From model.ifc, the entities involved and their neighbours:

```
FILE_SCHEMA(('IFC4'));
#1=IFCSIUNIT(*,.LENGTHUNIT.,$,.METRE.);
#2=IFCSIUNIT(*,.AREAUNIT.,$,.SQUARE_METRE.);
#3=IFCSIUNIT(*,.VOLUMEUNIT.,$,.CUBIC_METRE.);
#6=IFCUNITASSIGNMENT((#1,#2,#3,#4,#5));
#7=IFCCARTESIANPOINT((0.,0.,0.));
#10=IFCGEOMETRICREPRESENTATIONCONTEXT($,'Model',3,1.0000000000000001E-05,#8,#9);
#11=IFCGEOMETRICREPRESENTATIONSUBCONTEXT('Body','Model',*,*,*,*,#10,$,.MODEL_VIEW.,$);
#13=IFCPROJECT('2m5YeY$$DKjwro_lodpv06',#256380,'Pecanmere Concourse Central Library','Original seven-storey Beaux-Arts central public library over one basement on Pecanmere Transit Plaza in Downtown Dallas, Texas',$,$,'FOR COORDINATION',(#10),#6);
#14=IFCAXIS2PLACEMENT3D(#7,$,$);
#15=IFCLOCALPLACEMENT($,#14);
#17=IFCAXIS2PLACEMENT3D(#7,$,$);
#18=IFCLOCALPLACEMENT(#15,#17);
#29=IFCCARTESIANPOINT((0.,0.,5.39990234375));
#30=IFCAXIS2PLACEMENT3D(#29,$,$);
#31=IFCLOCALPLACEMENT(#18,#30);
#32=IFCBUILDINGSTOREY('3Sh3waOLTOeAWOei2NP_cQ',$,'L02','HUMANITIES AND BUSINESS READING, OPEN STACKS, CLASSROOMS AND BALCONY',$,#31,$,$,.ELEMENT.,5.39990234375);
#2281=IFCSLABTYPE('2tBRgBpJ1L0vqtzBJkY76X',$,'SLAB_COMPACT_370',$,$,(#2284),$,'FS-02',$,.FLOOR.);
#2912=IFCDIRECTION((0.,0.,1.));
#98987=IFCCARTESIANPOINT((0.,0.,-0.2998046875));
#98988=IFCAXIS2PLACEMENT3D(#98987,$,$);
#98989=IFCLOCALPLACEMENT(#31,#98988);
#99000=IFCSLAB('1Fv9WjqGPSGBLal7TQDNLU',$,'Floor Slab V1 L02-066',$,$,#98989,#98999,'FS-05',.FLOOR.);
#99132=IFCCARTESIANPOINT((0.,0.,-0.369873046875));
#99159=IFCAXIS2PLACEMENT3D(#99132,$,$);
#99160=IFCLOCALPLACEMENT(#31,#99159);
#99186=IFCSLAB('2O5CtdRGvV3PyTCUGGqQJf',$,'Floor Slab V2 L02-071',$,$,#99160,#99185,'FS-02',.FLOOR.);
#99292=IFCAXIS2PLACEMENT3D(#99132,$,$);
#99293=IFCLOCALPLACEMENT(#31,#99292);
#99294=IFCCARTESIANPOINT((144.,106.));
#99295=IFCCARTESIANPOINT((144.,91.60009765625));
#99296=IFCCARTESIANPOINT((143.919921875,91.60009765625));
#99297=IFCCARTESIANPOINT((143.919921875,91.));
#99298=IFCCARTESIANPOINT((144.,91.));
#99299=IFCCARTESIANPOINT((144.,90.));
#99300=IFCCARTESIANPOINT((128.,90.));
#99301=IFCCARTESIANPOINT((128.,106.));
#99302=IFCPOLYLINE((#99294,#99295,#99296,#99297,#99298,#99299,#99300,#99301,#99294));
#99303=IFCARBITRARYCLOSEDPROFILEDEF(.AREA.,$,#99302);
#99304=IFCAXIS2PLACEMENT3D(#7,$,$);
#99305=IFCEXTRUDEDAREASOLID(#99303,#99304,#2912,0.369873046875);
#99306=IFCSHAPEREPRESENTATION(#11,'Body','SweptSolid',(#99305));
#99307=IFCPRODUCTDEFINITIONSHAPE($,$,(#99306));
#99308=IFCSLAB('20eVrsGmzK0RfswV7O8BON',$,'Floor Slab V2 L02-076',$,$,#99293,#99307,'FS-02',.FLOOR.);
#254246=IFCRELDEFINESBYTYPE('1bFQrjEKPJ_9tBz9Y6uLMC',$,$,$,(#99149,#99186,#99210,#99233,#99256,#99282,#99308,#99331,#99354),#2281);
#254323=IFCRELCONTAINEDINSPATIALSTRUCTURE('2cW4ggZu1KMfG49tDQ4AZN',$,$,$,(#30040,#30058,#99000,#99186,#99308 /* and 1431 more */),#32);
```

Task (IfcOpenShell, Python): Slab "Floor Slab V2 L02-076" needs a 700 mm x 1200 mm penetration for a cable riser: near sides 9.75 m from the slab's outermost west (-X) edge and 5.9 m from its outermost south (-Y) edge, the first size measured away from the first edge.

```python
import numpy as np
import ifcopenshell
import ifcopenshell.api.feature
import ifcopenshell.api.geometry
import ifcopenshell.api.root
import ifcopenshell.geom
import ifcopenshell.util.placement
import ifcopenshell.util.representation
import ifcopenshell.util.shape
import ifcopenshell.util.unit

model = ifcopenshell.open("model.ifc")
unit_scale = ifcopenshell.util.unit.calculate_unit_scale(model)
settings = ifcopenshell.geom.settings()


def volume(element):
    """Net volume in cubic metres, openings subtracted."""
    shape = ifcopenshell.geom.create_shape(settings, element)
    return ifcopenshell.util.shape.get_volume(shape.geometry)


slab = model.by_guid("20eVrsGmzK0RfswV7O8BON")
before = volume(slab)

# Extent in the slab's own axes, in metres. The edges named are its -X and -Y sides.
slab_shape = ifcopenshell.geom.create_shape(settings, slab)
vertices = ifcopenshell.util.shape.get_vertices(slab_shape.geometry)
x_min, y_min, bottom = vertices.min(axis=0)
top = vertices[:, 2].max()

opening = ifcopenshell.api.root.create_entity(model, ifc_class="IfcOpeningElement", name="Cable riser opening", predefined_type="OPENING")
context = ifcopenshell.util.representation.get_context(model, "Model", "Body", "MODEL_VIEW")
width, depth = 0.7, 1.2
outline = [(0.0, 0.0), (width, 0.0), (width, depth), (0.0, depth), (0.0, 0.0)]
# Overshoot both faces by 50 mm so the cut is clean.
shape = ifcopenshell.api.geometry.add_slab_representation(
    model, context=context, depth=top - bottom + 0.1, polyline=outline
)
ifcopenshell.api.geometry.assign_representation(model, product=opening, representation=shape)

matrix = ifcopenshell.util.placement.get_local_placement(slab.ObjectPlacement)
matrix[:, 3] = matrix @ np.append(np.array([x_min + 9.75, y_min + 5.9, bottom - 0.05]) / unit_scale, 1.0)
ifcopenshell.api.geometry.edit_object_placement(model, product=opening, matrix=matrix, is_si=False)
ifcopenshell.api.feature.add_feature(model, feature=opening, element=slab)

after = volume(slab)

print(f"slab volume {before:.3f} -> {after:.3f} m3")

model.write("model-out.ifc")
```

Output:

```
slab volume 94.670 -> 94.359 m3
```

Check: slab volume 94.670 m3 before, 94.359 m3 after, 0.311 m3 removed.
